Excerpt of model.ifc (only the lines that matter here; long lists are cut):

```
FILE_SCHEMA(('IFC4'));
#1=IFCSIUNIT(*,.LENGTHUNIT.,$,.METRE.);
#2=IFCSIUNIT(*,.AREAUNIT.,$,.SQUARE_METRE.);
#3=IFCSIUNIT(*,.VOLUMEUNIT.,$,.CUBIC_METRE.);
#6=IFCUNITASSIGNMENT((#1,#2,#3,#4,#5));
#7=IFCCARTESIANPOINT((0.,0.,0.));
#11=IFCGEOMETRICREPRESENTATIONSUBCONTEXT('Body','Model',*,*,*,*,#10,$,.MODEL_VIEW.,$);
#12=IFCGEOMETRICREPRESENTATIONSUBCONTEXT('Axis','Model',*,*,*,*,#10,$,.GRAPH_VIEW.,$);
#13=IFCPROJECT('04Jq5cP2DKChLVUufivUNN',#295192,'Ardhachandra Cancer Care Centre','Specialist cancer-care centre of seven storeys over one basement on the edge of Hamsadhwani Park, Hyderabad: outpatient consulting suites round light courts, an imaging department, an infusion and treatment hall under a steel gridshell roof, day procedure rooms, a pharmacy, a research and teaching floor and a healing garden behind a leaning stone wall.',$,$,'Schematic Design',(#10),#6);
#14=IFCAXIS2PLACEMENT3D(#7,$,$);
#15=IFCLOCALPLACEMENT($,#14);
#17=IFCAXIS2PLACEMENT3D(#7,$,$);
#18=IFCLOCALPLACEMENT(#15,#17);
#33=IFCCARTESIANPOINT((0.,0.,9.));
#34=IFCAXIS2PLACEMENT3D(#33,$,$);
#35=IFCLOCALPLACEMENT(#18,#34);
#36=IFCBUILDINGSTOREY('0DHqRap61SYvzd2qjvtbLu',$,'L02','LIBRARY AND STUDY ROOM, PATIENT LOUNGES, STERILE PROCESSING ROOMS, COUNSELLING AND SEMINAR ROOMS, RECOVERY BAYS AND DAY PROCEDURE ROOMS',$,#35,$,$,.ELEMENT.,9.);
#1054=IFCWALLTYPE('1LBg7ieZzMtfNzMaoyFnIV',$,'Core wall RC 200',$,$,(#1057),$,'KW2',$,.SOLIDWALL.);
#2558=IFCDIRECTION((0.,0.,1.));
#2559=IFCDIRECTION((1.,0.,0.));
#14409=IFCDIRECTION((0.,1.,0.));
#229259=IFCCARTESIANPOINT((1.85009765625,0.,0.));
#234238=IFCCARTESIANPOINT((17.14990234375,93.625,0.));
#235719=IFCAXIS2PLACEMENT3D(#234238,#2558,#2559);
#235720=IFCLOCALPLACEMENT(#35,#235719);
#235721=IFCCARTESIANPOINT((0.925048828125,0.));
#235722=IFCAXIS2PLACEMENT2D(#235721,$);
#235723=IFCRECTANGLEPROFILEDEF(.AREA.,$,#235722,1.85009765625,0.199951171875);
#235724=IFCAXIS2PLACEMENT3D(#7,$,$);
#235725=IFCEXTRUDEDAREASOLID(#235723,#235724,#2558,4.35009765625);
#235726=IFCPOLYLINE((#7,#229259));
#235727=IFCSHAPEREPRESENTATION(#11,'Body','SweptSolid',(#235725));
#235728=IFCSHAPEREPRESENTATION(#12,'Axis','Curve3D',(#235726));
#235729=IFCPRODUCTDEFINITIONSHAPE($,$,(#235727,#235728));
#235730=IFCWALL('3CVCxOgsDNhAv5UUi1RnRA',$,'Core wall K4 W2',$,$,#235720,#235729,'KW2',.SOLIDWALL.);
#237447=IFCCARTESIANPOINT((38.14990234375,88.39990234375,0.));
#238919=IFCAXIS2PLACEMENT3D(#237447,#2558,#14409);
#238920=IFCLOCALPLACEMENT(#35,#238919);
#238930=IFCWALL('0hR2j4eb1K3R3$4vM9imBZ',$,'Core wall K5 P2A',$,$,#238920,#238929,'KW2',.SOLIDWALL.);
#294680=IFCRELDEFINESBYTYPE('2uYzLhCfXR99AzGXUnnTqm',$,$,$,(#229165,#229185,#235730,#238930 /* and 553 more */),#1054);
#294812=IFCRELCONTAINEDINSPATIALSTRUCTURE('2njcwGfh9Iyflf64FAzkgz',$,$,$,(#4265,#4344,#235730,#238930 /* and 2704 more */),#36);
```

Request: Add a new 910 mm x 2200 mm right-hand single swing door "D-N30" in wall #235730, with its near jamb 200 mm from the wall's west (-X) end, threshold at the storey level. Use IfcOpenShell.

```python
import numpy as np
import ifcopenshell
import ifcopenshell.api.feature
import ifcopenshell.api.geometry
import ifcopenshell.api.root
import ifcopenshell.api.spatial
import ifcopenshell.geom
import ifcopenshell.util.element
import ifcopenshell.util.placement
import ifcopenshell.util.representation
import ifcopenshell.util.shape
import ifcopenshell.util.unit

model = ifcopenshell.open("model.ifc")
unit_scale = ifcopenshell.util.unit.calculate_unit_scale(model)
settings = ifcopenshell.geom.settings()


def volume(element):
    """Net volume in cubic metres, openings subtracted."""
    shape = ifcopenshell.geom.create_shape(settings, element)
    return ifcopenshell.util.shape.get_volume(shape.geometry)


wall = model.by_id(235730)
storey = ifcopenshell.util.element.get_container(wall, ifc_class="IfcBuildingStorey")
context = ifcopenshell.util.representation.get_context(model, "Model", "Body", "MODEL_VIEW")
before = volume(wall)

width, height, from_end, sill = 0.91, 2.2, 0.2, 0.0  # metres

# The wall runs along its own X axis, and the end named is its -X end.
wall_shape = ifcopenshell.geom.create_shape(settings, wall)
x, y, z = ifcopenshell.util.shape.get_vertices(wall_shape.geometry).T
start = x.min() + from_end
face, thickness = float(y.min()), float(y.max() - y.min())
wall_matrix = ifcopenshell.util.placement.get_local_placement(wall.ObjectPlacement)
level = ifcopenshell.util.placement.get_local_placement(storey.ObjectPlacement)[2, 3]


def in_wall(x, y):
    """Placement at x, y metres in the wall's axes, at sill height."""
    matrix = wall_matrix.copy()
    matrix[:, 3] = wall_matrix @ np.array([x / unit_scale, y / unit_scale, 0.0, 1.0])
    matrix[2, 3] = level + sill / unit_scale
    return matrix


# Opening: a box that overshoots both wall faces by 50 mm.
opening = ifcopenshell.api.root.create_entity(model, ifc_class="IfcOpeningElement", predefined_type="OPENING")
box = ifcopenshell.api.geometry.add_wall_representation(
    model, context=context, length=width, height=height, thickness=thickness + 0.1
)
ifcopenshell.api.geometry.assign_representation(model, product=opening, representation=box)
ifcopenshell.api.geometry.edit_object_placement(model, product=opening, matrix=in_wall(start, face - 0.05), is_si=False)
ifcopenshell.api.feature.add_feature(model, feature=opening, element=wall)

door = ifcopenshell.api.root.create_entity(model, ifc_class="IfcDoor", name="D-N30", predefined_type="DOOR")
door.OverallWidth, door.OverallHeight = width / unit_scale, height / unit_scale
door.OperationType = "SINGLE_SWING_RIGHT"
body = ifcopenshell.api.geometry.add_door_representation(
    model,
    context=context,
    overall_width=door.OverallWidth,
    overall_height=door.OverallHeight,
    operation_type="SINGLE_SWING_RIGHT",
    lining_properties={"LiningDepth": thickness / unit_scale, "ThresholdDepth": thickness / unit_scale},
)
ifcopenshell.api.geometry.assign_representation(model, product=door, representation=body)
ifcopenshell.api.spatial.assign_container(model, products=[door], relating_structure=storey)
ifcopenshell.api.feature.add_filling(model, opening=opening, element=door)

# The lining spans the wall, so the door starts at the wall face.
ifcopenshell.api.geometry.edit_object_placement(model, product=door, matrix=in_wall(start, face), is_si=False)

after = volume(wall)

print(f"wall volume {before:.3f} -> {after:.3f} m3")

model.write("model_edited.ifc")
```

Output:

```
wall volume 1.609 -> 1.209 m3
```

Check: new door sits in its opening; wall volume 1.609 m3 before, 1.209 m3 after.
